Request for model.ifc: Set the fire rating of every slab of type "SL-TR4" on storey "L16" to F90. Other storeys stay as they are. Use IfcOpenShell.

First a look at what the model holds.

```python
import ifcopenshell
import ifcopenshell.util.element

model = ifcopenshell.open("model.ifc")
print(model.schema)
storey = next(s for s in model.by_type("IfcBuildingStorey") if s.Name == "L16")
slabs = [e for e in ifcopenshell.util.element.get_decomposition(storey) if e.is_a("IfcSlab")]
seen = {}
for e in slabs:
    element_type = ifcopenshell.util.element.get_type(e)
    key = (element_type.Name if element_type != e and element_type else None, ifcopenshell.util.element.get_pset(e, "Pset_SlabCommon", "FireRating"))
    seen[key] = seen.get(key, 0) + 1
for (name, value), count in sorted(seen.items(), key=str):
    print(count, "x", name, "|", value)
```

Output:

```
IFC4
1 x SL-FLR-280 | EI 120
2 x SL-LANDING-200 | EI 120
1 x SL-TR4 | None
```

```python
import ifcopenshell
import ifcopenshell.api.pset
import ifcopenshell.util.element

model = ifcopenshell.open("model.ifc")

storey = next(s for s in model.by_type("IfcBuildingStorey") if s.Name == "L16")
slabs = [e for e in ifcopenshell.util.element.get_decomposition(storey) if e.is_a("IfcSlab")]

count = 0
for e in slabs:
    element_type = ifcopenshell.util.element.get_type(e)
    if element_type in (None, e) or element_type.Name != "SL-TR4":
        continue
    found = ifcopenshell.util.element.get_pset(e, "Pset_SlabCommon", should_inherit=False)
    if found:
        pset = model.by_id(found["id"])
        if len(ifcopenshell.util.element.get_elements_by_pset(pset)) > 1:
            pset = ifcopenshell.api.pset.unshare_pset(model, products=[e], pset=pset)[0]
    else:
        pset = ifcopenshell.api.pset.add_pset(model, product=e, name="Pset_SlabCommon")
    ifcopenshell.api.pset.edit_pset(model, pset=pset, properties={"FireRating": "F90"})
    count += 1

print(count, "slabs updated")

model.write("model_edited.ifc")
```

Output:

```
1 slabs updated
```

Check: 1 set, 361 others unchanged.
